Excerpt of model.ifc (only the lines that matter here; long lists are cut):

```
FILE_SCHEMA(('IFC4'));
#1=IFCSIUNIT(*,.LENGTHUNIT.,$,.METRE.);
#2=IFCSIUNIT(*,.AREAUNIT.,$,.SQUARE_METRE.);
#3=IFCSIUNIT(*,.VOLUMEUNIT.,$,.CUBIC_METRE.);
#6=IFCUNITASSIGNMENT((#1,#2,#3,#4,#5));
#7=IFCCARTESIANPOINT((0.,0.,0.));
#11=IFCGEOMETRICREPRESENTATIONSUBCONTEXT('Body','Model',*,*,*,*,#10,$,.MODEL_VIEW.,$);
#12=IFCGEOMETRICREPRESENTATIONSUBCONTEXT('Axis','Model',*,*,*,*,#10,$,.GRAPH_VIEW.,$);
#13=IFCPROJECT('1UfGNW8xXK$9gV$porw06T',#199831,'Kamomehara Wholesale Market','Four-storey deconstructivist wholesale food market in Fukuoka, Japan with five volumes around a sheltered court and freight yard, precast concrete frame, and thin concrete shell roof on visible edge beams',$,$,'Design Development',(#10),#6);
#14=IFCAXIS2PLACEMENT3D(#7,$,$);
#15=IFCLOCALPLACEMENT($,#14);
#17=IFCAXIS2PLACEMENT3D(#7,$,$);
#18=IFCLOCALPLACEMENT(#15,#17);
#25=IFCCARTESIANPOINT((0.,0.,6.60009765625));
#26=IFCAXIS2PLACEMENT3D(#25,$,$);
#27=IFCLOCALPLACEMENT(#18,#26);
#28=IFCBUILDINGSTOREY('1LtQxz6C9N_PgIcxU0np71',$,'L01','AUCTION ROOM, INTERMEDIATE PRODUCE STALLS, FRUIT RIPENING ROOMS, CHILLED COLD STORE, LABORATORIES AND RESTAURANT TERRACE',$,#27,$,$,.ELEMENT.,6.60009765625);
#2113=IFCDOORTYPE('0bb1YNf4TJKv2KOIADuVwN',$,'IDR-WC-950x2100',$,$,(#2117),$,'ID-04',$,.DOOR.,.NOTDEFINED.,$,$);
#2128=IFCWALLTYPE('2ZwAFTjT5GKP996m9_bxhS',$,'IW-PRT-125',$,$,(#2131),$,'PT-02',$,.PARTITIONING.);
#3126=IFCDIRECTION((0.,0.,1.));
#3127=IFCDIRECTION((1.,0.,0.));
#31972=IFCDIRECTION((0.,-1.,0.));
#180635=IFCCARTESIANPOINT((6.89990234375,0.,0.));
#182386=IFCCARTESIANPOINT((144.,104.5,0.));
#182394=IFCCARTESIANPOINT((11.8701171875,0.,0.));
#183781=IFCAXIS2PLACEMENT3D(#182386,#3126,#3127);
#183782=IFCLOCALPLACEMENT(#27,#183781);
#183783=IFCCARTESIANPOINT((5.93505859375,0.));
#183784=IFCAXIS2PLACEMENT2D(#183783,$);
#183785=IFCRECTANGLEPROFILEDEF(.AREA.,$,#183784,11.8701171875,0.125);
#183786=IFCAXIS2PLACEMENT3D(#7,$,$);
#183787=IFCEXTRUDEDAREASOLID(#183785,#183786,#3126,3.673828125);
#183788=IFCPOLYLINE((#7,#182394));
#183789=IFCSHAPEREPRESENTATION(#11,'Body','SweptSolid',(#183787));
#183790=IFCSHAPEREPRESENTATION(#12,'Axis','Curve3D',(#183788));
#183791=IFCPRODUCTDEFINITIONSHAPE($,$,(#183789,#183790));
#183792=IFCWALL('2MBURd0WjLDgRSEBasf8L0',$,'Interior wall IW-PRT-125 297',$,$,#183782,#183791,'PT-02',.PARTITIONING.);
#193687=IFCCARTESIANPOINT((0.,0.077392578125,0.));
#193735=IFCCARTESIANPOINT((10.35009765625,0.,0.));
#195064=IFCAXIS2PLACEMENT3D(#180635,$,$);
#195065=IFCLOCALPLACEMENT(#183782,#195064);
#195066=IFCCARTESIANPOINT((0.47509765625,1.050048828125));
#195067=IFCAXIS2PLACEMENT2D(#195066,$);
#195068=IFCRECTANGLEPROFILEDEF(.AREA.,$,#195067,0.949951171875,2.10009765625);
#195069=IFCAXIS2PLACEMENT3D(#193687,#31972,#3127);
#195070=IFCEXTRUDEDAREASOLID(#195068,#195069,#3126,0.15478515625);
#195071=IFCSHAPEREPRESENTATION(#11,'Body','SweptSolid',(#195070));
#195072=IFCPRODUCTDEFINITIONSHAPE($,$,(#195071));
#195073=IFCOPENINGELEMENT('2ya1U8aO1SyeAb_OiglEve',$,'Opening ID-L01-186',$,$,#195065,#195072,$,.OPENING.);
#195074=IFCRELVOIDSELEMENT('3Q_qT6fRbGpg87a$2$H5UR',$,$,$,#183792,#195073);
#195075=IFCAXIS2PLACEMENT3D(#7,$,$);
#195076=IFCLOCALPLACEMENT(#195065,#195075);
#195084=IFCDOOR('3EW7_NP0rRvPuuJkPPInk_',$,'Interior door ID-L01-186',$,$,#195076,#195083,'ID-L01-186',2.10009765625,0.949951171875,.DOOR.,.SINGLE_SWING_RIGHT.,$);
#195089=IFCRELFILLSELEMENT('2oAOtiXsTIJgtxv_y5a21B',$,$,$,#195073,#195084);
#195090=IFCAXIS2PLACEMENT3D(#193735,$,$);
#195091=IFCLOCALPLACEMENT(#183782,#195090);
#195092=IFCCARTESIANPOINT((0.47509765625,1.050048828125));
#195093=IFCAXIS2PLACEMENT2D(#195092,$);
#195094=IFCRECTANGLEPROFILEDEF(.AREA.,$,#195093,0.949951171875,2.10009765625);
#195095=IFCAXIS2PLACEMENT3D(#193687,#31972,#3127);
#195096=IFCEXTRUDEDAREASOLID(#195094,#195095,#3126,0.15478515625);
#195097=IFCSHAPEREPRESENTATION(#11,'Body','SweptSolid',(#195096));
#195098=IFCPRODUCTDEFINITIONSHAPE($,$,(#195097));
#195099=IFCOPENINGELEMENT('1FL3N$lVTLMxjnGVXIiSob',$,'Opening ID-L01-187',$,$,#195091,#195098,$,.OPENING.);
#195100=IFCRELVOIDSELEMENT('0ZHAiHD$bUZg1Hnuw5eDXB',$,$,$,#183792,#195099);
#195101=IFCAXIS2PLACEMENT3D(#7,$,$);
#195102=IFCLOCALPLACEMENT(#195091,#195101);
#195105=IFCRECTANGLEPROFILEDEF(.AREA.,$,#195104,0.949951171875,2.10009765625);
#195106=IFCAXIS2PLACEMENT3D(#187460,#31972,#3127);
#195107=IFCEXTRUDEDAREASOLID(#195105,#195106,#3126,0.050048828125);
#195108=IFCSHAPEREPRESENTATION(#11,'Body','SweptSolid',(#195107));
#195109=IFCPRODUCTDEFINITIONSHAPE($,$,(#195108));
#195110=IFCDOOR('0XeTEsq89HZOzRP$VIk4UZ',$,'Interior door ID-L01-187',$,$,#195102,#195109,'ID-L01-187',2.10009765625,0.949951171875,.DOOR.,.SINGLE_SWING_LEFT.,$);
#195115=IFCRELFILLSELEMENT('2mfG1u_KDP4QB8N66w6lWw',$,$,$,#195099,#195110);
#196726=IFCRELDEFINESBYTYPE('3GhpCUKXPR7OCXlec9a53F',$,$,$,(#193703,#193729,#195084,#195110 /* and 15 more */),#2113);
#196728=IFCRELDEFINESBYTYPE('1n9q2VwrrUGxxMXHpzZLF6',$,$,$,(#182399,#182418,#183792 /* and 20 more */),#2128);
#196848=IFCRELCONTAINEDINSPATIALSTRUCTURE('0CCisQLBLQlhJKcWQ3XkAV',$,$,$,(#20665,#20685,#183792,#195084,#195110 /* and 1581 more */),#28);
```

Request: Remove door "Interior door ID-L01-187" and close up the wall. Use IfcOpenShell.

```python
import ifcopenshell
import ifcopenshell.api.feature
import ifcopenshell.api.root
import ifcopenshell.geom
import ifcopenshell.util.shape

model = ifcopenshell.open("model.ifc")
settings = ifcopenshell.geom.settings()


def volume(element):
    """Net volume in cubic metres, openings subtracted."""
    shape = ifcopenshell.geom.create_shape(settings, element)
    return ifcopenshell.util.shape.get_volume(shape.geometry)


door = model.by_guid("0XeTEsq89HZOzRP$VIk4UZ")
opening = door.FillsVoids[0].RelatingOpeningElement
wall = opening.VoidsElements[0].RelatingBuildingElement
before = volume(wall)

ifcopenshell.api.root.remove_product(model, product=door)
ifcopenshell.api.feature.remove_feature(model, feature=opening)

after = volume(wall)

print(f"wall volume {before:.3f} -> {after:.3f} m3")

model.write("model_edited.ifc")
```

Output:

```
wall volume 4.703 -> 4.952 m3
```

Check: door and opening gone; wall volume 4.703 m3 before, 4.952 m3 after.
